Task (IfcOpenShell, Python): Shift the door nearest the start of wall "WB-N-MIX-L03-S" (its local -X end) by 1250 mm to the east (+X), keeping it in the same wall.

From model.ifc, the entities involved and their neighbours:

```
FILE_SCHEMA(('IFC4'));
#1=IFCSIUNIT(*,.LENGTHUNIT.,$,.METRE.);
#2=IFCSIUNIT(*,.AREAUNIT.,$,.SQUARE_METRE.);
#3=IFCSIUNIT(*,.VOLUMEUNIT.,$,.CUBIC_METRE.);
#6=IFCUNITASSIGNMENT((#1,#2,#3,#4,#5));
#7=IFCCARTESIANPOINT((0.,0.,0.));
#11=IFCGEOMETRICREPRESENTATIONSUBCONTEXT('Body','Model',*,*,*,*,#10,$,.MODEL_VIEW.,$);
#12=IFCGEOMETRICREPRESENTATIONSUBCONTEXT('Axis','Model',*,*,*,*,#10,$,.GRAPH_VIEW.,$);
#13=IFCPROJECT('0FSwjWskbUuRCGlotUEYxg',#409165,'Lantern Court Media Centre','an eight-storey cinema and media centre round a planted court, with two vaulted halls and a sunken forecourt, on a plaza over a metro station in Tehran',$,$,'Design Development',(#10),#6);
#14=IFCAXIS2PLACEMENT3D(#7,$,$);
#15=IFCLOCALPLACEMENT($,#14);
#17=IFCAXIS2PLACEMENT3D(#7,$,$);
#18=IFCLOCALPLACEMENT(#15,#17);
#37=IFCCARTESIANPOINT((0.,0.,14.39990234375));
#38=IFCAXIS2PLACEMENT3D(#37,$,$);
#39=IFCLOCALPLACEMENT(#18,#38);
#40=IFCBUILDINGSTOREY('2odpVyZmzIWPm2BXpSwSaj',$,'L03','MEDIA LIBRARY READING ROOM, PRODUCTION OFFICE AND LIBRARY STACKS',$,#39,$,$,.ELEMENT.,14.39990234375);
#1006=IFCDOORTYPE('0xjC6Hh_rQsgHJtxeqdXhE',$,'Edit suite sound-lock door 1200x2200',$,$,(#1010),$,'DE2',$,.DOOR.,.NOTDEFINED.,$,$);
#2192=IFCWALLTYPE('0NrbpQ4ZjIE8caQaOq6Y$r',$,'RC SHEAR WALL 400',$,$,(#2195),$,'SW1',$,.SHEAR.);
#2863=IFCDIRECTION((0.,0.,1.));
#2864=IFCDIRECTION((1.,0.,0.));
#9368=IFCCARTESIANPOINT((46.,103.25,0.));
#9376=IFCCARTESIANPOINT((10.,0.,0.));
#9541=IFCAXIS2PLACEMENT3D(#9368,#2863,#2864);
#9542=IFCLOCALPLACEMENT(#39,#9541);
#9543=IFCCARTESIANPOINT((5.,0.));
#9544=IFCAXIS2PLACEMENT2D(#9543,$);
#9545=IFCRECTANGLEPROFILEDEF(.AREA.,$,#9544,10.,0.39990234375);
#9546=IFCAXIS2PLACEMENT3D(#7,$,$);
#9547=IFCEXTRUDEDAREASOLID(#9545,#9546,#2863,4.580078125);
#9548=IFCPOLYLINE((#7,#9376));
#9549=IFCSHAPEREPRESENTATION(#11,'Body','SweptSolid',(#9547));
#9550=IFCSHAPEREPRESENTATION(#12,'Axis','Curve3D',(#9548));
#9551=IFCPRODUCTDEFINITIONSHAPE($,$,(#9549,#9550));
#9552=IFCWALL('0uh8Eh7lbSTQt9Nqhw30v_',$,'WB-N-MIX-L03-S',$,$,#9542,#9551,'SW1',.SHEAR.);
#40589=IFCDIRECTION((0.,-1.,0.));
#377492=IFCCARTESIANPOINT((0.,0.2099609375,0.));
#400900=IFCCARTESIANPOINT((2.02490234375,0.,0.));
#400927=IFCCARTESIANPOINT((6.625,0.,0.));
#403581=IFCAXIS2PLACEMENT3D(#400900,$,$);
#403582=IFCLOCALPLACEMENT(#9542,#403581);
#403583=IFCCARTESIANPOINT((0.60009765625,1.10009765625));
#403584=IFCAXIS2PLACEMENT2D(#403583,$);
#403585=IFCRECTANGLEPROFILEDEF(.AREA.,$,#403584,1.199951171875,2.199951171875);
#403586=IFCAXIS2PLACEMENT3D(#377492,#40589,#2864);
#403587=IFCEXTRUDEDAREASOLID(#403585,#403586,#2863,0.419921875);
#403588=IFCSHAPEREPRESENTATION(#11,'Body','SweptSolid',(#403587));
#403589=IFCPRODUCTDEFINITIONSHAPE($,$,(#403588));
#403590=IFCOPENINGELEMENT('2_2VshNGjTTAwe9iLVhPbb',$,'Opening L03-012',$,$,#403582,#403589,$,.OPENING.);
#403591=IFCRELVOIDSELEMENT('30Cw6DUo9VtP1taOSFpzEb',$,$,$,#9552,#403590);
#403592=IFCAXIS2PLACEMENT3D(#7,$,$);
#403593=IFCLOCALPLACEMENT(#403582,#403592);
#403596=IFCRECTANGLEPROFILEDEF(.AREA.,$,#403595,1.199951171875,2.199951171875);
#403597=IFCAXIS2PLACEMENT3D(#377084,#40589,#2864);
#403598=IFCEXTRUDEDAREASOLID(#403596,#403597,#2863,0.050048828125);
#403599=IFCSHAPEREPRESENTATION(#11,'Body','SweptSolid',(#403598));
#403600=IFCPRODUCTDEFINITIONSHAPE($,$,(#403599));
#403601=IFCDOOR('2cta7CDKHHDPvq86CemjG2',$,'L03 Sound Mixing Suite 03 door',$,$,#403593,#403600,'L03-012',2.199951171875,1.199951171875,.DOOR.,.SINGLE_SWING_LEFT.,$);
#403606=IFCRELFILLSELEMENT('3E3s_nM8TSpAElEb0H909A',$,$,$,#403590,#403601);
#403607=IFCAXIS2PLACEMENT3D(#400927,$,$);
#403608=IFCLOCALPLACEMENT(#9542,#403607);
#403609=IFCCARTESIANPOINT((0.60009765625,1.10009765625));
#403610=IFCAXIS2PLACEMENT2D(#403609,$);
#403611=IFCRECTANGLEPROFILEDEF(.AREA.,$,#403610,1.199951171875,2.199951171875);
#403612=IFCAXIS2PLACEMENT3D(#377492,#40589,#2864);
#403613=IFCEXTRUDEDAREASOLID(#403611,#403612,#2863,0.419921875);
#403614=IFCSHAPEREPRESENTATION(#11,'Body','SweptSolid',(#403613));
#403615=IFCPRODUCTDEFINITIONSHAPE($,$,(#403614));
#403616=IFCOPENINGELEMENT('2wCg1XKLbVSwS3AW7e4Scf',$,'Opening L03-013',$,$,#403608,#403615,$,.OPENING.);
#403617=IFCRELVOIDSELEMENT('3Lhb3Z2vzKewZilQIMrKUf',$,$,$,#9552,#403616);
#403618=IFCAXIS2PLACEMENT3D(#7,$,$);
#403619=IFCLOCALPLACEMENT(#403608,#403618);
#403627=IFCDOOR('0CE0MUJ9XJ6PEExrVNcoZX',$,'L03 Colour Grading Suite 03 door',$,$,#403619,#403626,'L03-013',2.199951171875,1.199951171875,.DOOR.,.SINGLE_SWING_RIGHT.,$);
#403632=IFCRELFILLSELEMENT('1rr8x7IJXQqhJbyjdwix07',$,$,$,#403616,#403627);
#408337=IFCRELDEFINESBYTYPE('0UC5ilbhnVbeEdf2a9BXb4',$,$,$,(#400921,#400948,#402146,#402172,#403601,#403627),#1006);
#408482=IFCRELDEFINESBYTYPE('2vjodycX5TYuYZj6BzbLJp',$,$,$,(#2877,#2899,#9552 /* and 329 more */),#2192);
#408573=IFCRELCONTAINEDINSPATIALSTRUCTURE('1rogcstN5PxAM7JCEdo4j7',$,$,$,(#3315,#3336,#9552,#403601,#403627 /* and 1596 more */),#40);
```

```python
import ifcopenshell
import ifcopenshell.api.geometry
import ifcopenshell.util.placement
import ifcopenshell.util.unit

model = ifcopenshell.open("model.ifc")
unit_scale = ifcopenshell.util.unit.calculate_unit_scale(model)

door = model.by_guid("2cta7CDKHHDPvq86CemjG2")
opening = door.FillsVoids[0].RelatingOpeningElement
wall = opening.VoidsElements[0].RelatingBuildingElement

wall_matrix = ifcopenshell.util.placement.get_local_placement(wall.ObjectPlacement)
shift = wall_matrix[:3, 0] * 1.25 / unit_scale
before = ifcopenshell.util.placement.get_local_placement(door.ObjectPlacement)[:3, 3].copy()

# The door is placed relative to its opening, so it follows when the opening moves.
matrix = ifcopenshell.util.placement.get_local_placement(opening.ObjectPlacement)
matrix[:3, 3] += shift
ifcopenshell.api.geometry.edit_object_placement(
    model, product=opening, matrix=matrix, is_si=False, should_transform_children=True
)

after = ifcopenshell.util.placement.get_local_placement(door.ObjectPlacement)[:3, 3]
print("door moved by", (after - before).round(3) + 0.0)

model.write("model_rev.ifc")
```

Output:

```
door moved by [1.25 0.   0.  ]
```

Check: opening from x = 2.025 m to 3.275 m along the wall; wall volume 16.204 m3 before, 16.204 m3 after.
